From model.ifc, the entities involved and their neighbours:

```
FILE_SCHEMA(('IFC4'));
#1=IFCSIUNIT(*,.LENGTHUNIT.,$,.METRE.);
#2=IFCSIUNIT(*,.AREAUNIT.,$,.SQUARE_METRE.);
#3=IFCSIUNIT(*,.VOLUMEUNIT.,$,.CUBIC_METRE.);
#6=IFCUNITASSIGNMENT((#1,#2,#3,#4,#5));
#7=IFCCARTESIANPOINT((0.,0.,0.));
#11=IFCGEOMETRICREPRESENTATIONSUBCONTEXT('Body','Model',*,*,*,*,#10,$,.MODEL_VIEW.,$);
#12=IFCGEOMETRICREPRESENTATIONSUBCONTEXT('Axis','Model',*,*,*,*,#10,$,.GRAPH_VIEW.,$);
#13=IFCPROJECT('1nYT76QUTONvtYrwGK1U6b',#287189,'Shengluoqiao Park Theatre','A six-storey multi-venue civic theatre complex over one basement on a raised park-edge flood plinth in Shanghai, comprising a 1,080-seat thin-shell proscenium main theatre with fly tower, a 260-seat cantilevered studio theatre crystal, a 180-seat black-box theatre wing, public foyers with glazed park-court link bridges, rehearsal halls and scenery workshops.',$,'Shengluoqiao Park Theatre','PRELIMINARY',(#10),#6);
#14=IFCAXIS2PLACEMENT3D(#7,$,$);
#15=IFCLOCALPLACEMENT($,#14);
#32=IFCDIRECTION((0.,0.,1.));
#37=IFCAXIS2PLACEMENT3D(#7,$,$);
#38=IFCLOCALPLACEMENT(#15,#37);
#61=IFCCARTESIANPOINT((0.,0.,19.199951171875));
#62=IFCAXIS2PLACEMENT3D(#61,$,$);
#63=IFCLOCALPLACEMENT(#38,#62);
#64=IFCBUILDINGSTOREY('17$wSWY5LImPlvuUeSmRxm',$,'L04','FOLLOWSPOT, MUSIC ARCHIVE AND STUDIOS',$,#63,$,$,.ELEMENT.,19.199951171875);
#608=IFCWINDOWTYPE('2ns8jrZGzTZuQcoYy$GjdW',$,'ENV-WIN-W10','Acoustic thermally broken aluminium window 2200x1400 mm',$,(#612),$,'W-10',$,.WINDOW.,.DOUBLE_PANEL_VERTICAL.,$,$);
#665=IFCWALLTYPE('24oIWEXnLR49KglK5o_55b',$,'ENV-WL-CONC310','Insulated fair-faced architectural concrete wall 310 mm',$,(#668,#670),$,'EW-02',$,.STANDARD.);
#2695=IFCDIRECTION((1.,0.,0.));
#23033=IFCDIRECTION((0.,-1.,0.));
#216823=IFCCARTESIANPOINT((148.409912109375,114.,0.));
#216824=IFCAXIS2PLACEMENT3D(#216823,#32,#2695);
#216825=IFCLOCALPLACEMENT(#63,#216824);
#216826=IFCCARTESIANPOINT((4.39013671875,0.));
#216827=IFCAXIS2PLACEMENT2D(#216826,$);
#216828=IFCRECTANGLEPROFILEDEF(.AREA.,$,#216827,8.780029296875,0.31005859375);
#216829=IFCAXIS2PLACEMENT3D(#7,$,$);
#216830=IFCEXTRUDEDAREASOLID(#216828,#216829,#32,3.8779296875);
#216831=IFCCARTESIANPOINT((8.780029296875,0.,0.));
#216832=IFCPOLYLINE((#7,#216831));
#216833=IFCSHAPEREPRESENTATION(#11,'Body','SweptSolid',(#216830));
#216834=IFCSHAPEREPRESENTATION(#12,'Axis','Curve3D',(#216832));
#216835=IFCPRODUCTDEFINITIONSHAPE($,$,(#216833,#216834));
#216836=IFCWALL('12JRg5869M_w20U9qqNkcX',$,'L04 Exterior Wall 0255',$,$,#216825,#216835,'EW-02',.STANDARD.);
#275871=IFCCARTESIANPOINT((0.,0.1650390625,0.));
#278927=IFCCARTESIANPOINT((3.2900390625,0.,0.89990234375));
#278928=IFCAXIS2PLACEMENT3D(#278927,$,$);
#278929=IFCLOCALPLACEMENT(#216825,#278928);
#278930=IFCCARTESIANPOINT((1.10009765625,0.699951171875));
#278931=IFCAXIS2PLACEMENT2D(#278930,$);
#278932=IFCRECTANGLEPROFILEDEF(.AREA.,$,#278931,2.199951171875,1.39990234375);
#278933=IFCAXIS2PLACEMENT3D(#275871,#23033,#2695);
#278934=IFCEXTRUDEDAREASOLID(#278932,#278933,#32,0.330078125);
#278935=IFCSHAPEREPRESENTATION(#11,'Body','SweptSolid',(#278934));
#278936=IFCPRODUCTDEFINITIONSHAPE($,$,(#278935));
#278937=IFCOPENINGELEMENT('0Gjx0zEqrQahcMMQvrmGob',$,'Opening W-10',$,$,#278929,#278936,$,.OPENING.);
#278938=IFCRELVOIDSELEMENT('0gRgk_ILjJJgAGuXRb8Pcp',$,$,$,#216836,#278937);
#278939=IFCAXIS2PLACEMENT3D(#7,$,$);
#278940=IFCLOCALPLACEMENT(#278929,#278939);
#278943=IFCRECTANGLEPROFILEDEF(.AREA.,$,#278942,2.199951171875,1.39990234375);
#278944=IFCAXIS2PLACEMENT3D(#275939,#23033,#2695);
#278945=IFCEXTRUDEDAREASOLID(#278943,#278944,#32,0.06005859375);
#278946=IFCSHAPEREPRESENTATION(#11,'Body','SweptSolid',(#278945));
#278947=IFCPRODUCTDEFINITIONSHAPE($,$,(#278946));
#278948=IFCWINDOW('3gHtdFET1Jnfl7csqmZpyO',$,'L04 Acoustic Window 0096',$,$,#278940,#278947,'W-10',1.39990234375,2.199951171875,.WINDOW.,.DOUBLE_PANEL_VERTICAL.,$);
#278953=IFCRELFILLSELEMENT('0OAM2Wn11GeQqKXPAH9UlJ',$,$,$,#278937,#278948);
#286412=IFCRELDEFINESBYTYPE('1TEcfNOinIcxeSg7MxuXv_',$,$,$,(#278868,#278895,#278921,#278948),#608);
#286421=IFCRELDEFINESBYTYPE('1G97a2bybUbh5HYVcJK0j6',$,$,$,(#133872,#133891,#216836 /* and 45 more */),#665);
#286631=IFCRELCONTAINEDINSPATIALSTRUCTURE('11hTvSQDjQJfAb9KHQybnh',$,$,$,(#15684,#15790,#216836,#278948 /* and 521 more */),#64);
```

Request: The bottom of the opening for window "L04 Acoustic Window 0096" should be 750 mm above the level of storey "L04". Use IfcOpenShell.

```python
import numpy as np
import ifcopenshell
import ifcopenshell.api.geometry
import ifcopenshell.geom
import ifcopenshell.util.element
import ifcopenshell.util.placement
import ifcopenshell.util.shape
import ifcopenshell.util.unit

model = ifcopenshell.open("model.ifc")
unit_scale = ifcopenshell.util.unit.calculate_unit_scale(model)

window = model.by_guid("3gHtdFET1Jnfl7csqmZpyO")
opening = window.FillsVoids[0].RelatingOpeningElement
storey = ifcopenshell.util.element.get_container(window, ifc_class="IfcBuildingStorey")
level = ifcopenshell.util.placement.get_local_placement(storey.ObjectPlacement)[2, 3]

# The opening's origin need not be at the sill, so measure its lowest point.
shape = ifcopenshell.geom.create_shape(ifcopenshell.geom.settings(), opening)
bottom = ifcopenshell.util.shape.get_shape_bottom_elevation(shape, shape.geometry) / unit_scale
dz = level + 0.75 / unit_scale - bottom

shift = np.array([0.0, 0.0, dz])
# The window is placed relative to its opening, so it follows when the opening moves.
matrix = ifcopenshell.util.placement.get_local_placement(opening.ObjectPlacement)
matrix[:3, 3] += shift
ifcopenshell.api.geometry.edit_object_placement(
    model, product=opening, matrix=matrix, is_si=False, should_transform_children=True
)

print(f"moved by {dz * unit_scale:+.3f} m")

model.write("model_rev.ifc")
```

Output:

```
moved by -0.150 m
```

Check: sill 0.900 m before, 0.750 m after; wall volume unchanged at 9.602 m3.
